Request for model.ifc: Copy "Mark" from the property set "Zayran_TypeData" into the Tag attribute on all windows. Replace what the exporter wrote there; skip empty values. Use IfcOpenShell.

First a look at what the model holds.

```python
import ifcopenshell
import ifcopenshell.util.element

model = ifcopenshell.open("model.ifc")
print(model.schema)
windows = model.by_type("IfcWindow")
print(len(windows), "windows")
for e in windows[:8]:
    source = ifcopenshell.util.element.get_pset(e, "Zayran_TypeData", "Mark")
    target = e.Tag
    print(e.id(), repr(source), repr(target), sep=" | ")
```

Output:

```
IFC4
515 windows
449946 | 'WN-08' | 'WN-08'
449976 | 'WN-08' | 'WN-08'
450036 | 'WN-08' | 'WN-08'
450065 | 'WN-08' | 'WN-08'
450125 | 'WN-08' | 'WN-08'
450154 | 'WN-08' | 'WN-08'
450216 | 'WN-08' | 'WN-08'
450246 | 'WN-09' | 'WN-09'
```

```python
import ifcopenshell
import ifcopenshell.util.element

model = ifcopenshell.open("model.ifc")

count = 0
for e in model.by_type("IfcWindow"):
    value = ifcopenshell.util.element.get_pset(e, "Zayran_TypeData", "Mark")
    current = e.Tag
    if not value or not value.strip() or current == value:
        continue
    e.Tag = value
    count += 1

print(count, "windows updated")

model.write("model-out.ifc")
```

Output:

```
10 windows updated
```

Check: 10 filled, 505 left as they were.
